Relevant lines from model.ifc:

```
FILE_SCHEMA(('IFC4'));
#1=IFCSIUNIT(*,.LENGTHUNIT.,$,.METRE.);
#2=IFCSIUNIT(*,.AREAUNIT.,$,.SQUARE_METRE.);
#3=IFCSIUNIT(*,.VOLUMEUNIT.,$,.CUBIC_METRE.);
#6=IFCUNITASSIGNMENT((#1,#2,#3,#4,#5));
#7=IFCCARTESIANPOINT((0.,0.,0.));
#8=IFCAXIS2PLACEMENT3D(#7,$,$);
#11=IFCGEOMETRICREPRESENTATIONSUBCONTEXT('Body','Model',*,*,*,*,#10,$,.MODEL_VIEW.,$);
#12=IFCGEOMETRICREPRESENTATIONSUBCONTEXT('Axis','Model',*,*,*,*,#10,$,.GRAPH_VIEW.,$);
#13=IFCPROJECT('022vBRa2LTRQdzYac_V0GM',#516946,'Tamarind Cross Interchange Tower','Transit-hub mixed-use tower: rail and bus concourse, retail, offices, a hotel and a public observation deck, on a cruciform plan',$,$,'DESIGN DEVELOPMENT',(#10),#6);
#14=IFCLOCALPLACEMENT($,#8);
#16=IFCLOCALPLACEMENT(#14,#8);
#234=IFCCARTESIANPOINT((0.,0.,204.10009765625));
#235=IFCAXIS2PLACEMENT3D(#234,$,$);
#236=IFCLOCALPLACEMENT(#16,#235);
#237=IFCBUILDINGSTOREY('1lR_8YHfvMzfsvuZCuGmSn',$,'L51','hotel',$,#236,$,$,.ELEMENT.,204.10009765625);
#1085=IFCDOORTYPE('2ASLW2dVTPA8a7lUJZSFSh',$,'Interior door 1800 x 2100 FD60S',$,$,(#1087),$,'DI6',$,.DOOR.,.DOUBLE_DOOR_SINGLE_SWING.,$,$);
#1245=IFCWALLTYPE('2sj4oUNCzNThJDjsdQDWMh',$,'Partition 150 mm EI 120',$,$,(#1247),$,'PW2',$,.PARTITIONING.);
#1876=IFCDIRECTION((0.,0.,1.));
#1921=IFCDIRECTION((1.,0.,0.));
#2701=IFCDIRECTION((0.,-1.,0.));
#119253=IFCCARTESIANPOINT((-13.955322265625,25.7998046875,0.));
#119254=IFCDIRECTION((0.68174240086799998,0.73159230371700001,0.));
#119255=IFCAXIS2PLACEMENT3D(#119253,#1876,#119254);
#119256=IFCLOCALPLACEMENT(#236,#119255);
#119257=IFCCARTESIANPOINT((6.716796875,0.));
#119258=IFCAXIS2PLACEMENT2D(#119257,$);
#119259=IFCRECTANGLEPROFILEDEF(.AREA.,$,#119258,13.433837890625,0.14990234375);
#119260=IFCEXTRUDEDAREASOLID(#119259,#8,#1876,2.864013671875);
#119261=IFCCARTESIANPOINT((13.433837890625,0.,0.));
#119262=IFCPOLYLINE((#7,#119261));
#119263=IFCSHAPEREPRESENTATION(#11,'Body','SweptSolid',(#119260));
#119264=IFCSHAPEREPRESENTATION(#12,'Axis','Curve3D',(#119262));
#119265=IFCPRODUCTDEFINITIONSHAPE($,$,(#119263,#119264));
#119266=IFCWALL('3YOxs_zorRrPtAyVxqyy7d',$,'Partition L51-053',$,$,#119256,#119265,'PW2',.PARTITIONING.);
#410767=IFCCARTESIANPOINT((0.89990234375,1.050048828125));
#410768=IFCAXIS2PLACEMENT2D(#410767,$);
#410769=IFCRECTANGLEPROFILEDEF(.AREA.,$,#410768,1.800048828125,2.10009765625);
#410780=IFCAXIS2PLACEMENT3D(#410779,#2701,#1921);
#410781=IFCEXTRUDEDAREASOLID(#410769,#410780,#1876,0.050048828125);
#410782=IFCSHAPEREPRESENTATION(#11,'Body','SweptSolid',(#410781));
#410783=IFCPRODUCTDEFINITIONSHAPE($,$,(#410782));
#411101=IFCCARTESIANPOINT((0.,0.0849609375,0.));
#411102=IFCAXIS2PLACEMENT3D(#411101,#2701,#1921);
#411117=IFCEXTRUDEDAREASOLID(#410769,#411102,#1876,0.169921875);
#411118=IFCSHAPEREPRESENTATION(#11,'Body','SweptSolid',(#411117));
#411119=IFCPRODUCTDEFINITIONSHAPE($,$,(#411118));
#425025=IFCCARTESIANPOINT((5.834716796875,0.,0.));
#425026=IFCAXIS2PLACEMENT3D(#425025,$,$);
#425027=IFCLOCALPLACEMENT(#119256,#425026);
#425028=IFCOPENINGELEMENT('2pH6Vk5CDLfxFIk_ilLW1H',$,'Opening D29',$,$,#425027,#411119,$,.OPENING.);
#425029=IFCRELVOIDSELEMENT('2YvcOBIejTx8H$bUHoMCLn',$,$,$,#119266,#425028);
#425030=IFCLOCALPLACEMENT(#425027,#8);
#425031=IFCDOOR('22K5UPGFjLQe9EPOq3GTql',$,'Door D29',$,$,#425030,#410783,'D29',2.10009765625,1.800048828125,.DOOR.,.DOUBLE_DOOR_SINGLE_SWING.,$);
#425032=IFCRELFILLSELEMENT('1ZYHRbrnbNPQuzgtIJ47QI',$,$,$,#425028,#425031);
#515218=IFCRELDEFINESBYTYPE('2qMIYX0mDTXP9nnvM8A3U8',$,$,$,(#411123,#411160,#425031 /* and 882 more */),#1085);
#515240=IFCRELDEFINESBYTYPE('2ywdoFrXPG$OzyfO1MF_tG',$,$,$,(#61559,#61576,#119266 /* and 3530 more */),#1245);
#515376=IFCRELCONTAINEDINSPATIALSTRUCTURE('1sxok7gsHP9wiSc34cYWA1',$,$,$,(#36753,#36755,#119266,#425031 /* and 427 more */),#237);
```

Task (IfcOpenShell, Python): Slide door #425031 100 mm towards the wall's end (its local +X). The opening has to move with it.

```python
import ifcopenshell
import ifcopenshell.api.geometry
import ifcopenshell.util.placement
import ifcopenshell.util.unit

model = ifcopenshell.open("model.ifc")
unit_scale = ifcopenshell.util.unit.calculate_unit_scale(model)

door = model.by_guid("22K5UPGFjLQe9EPOq3GTql")
opening = door.FillsVoids[0].RelatingOpeningElement
wall = opening.VoidsElements[0].RelatingBuildingElement

wall_matrix = ifcopenshell.util.placement.get_local_placement(wall.ObjectPlacement)
shift = wall_matrix[:3, 0] * 0.1 / unit_scale
before = ifcopenshell.util.placement.get_local_placement(door.ObjectPlacement)[:3, 3].copy()

# The door is placed relative to its opening, so it follows when the opening moves.
matrix = ifcopenshell.util.placement.get_local_placement(opening.ObjectPlacement)
matrix[:3, 3] += shift
ifcopenshell.api.geometry.edit_object_placement(
    model, product=opening, matrix=matrix, is_si=False, should_transform_children=True
)

after = ifcopenshell.util.placement.get_local_placement(door.ObjectPlacement)[:3, 3]
print("door moved by", (after - before).round(3) + 0.0)

model.write("model-out.ifc")
```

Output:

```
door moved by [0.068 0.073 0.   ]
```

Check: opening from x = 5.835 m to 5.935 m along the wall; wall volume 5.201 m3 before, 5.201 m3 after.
